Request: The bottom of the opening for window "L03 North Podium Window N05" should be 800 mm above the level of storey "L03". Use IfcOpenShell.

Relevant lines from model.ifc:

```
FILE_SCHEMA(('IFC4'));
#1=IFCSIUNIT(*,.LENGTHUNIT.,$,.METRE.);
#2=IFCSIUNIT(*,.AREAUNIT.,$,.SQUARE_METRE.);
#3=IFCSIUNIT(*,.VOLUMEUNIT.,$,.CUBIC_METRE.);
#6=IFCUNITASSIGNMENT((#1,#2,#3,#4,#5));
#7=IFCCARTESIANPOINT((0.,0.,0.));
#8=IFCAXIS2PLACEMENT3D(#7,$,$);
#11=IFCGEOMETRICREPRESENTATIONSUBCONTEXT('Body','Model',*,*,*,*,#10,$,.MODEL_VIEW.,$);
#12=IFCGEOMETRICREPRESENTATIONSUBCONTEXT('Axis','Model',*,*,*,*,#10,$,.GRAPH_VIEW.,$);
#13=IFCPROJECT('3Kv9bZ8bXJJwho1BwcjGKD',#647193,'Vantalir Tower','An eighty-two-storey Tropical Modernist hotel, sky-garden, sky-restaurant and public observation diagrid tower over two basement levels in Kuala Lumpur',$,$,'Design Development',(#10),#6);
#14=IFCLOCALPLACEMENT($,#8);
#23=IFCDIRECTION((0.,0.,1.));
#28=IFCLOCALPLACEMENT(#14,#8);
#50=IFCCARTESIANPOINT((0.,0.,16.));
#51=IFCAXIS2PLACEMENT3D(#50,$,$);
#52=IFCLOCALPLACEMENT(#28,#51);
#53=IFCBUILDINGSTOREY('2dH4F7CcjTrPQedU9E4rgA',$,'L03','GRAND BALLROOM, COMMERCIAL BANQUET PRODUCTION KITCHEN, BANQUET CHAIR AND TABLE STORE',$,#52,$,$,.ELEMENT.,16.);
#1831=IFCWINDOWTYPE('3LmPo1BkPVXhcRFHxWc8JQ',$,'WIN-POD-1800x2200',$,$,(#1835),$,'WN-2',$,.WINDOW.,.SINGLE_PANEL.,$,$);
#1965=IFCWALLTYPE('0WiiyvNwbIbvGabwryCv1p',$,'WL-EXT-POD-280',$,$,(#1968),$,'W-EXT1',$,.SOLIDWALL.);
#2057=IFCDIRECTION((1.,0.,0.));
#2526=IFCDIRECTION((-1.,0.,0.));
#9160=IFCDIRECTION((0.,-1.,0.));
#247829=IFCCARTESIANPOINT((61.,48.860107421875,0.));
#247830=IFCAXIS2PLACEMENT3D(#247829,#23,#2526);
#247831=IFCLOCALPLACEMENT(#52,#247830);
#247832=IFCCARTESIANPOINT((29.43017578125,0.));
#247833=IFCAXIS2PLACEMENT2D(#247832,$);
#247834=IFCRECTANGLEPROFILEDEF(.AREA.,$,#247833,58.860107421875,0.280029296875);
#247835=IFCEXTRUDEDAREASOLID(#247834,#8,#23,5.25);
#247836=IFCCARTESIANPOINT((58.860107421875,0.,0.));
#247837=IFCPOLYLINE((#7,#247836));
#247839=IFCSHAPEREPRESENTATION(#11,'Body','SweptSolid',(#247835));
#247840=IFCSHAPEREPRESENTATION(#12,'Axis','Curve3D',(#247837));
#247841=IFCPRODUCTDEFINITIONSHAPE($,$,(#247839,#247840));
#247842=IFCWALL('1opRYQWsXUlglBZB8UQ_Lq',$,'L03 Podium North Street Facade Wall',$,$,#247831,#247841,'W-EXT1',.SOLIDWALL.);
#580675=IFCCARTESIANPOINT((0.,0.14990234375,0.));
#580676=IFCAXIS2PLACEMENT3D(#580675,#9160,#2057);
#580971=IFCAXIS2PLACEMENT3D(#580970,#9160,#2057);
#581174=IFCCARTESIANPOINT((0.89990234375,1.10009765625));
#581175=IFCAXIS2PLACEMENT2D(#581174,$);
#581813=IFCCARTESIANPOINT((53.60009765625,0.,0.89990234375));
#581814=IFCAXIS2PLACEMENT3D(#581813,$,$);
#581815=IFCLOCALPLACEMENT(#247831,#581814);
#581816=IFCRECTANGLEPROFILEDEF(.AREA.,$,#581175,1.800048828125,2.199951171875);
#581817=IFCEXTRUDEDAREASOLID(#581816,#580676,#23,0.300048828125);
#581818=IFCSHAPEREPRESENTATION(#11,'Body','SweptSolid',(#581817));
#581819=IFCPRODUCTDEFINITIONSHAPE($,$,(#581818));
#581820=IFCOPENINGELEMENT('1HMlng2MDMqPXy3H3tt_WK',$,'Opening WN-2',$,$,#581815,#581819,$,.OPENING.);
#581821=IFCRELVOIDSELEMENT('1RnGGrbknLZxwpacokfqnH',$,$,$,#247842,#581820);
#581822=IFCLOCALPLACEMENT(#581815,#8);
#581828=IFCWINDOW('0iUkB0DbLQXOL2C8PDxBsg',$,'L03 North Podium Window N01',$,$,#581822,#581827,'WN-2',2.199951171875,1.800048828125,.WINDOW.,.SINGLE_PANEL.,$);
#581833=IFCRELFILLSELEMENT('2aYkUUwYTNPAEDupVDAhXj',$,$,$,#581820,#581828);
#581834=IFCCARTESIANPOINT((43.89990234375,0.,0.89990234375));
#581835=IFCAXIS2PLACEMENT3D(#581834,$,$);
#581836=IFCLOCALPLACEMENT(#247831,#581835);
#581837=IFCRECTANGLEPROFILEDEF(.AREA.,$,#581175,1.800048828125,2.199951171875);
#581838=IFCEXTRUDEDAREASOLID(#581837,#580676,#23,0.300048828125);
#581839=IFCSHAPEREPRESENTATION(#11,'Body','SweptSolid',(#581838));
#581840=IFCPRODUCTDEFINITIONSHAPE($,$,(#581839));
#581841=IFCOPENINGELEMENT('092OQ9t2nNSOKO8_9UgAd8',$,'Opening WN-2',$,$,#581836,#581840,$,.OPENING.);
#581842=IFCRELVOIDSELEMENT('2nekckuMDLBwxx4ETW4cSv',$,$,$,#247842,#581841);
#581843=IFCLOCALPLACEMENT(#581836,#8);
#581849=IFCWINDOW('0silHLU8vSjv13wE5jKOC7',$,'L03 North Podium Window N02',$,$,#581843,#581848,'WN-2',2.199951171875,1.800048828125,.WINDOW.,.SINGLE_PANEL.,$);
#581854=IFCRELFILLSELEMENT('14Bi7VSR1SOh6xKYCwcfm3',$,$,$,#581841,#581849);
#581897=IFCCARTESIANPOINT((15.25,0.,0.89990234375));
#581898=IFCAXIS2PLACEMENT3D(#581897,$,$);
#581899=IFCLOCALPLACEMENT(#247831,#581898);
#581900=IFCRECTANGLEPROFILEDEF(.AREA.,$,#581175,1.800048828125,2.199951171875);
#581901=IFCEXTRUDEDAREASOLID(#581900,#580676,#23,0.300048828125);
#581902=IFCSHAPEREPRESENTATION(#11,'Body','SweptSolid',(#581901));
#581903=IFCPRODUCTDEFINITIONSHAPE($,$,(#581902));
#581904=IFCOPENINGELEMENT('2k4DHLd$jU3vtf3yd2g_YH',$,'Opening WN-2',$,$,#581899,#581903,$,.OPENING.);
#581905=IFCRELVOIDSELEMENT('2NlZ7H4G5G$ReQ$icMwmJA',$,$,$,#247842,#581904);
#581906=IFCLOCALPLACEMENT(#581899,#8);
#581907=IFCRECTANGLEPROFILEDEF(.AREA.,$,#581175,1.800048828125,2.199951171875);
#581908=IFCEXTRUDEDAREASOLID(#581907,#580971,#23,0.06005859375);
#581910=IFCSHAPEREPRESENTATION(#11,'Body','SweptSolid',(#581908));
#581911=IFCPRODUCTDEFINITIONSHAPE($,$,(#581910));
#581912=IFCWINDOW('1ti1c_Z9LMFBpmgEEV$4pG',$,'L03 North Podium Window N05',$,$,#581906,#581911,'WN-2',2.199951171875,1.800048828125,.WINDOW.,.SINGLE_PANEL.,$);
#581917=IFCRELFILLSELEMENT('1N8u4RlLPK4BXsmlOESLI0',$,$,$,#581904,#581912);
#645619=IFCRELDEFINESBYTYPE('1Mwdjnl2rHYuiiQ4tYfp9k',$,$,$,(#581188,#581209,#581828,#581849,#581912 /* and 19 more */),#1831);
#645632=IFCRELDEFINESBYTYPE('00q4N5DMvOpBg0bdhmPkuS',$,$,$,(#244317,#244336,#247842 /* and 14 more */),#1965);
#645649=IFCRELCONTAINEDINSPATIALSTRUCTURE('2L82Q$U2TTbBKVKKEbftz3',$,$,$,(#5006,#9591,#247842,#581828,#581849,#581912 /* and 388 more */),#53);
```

```python
import numpy as np
import ifcopenshell
import ifcopenshell.api.geometry
import ifcopenshell.geom
import ifcopenshell.util.element
import ifcopenshell.util.placement
import ifcopenshell.util.shape
import ifcopenshell.util.unit

model = ifcopenshell.open("model.ifc")
unit_scale = ifcopenshell.util.unit.calculate_unit_scale(model)

window = model.by_id(581912)
opening = window.FillsVoids[0].RelatingOpeningElement
storey = ifcopenshell.util.element.get_container(window, ifc_class="IfcBuildingStorey")
level = ifcopenshell.util.placement.get_local_placement(storey.ObjectPlacement)[2, 3]

# The opening's origin need not be at the sill, so measure its lowest point.
shape = ifcopenshell.geom.create_shape(ifcopenshell.geom.settings(), opening)
bottom = ifcopenshell.util.shape.get_shape_bottom_elevation(shape, shape.geometry) / unit_scale
dz = level + 0.8 / unit_scale - bottom

shift = np.array([0.0, 0.0, dz])
# The window is placed relative to its opening, so it follows when the opening moves.
matrix = ifcopenshell.util.placement.get_local_placement(opening.ObjectPlacement)
matrix[:3, 3] += shift
ifcopenshell.api.geometry.edit_object_placement(
    model, product=opening, matrix=matrix, is_si=False, should_transform_children=True
)

print(f"moved by {dz * unit_scale:+.3f} m")

model.write("model-out.ifc")
```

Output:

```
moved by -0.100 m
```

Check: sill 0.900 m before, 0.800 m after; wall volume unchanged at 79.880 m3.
